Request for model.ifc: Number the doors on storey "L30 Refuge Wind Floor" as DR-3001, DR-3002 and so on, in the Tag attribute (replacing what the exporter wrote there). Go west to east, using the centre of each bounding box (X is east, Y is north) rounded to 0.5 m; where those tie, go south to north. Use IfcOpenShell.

First a look at what the model holds.

```python
import ifcopenshell
import ifcopenshell.util.element
import ifcopenshell.util.placement

model = ifcopenshell.open("model.ifc")
print(model.schema)
storey = next(s for s in model.by_type("IfcBuildingStorey") if s.Name == "L30 Refuge Wind Floor")
doors = [e for e in ifcopenshell.util.element.get_decomposition(storey) if e.is_a("IfcDoor")]
for e in sorted(doors, key=lambda e: e.id()):
    origin = ifcopenshell.util.placement.get_local_placement(e.ObjectPlacement)[:3, 3]
    print(e.id(), e.Tag, e.Name, origin.round(2) + 0.0, sep=" | ")
```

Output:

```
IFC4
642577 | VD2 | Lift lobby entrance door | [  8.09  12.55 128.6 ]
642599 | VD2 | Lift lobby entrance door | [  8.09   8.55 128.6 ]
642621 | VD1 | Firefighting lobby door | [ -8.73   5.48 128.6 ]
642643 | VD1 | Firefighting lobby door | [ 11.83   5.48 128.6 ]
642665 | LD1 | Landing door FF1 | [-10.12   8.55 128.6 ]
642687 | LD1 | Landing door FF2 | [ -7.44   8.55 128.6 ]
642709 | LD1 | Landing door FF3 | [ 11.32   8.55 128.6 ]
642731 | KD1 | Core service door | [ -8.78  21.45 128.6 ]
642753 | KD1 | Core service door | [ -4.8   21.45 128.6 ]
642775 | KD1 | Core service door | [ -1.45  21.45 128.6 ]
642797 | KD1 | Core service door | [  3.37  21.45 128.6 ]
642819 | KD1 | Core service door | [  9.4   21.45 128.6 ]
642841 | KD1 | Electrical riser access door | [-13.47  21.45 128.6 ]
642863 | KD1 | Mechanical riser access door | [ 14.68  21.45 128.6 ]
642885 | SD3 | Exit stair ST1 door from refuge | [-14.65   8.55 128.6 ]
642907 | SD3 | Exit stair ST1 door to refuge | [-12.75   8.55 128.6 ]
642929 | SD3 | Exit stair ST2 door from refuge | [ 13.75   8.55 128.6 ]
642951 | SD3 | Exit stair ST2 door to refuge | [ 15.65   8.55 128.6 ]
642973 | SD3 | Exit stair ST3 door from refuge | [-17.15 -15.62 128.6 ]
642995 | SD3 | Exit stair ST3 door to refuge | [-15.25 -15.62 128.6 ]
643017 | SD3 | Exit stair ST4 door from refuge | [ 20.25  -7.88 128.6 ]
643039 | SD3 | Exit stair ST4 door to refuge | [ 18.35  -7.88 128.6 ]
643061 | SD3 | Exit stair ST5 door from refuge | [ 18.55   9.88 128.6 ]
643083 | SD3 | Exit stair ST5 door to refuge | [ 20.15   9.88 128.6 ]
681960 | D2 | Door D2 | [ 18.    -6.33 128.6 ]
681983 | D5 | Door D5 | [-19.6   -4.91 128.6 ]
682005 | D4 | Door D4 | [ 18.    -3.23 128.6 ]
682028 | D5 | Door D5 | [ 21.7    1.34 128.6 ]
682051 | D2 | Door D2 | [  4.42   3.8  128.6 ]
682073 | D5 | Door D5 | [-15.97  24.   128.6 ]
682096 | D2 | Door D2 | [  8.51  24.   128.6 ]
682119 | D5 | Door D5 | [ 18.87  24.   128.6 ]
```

```python
import ifcopenshell
import ifcopenshell.geom
import ifcopenshell.util.element
import ifcopenshell.util.shape

model = ifcopenshell.open("model.ifc")
settings = ifcopenshell.geom.settings()
settings.set("use-world-coords", True)


def centre(element):
    shape = ifcopenshell.geom.create_shape(settings, element)
    return ifcopenshell.util.shape.get_bbox_centroid(shape.geometry)


storey = next(s for s in model.by_type("IfcBuildingStorey") if s.Name == "L30 Refuge Wind Floor")
doors = [e for e in ifcopenshell.util.element.get_decomposition(storey) if e.is_a("IfcDoor")]

# Insertion points can sit at a corner or the storey origin, so sort by the geometry (in metres).
centres = {e: centre(e) for e in doors}
doors.sort(key=lambda e: (round(centres[e][0] / 0.5), centres[e][1]))

for i, e in enumerate(doors, start=1):
    number = f"DR-30{i:02d}"
    e.Tag = number
    print(e.id(), number)

model.write("model_edited.ifc")
```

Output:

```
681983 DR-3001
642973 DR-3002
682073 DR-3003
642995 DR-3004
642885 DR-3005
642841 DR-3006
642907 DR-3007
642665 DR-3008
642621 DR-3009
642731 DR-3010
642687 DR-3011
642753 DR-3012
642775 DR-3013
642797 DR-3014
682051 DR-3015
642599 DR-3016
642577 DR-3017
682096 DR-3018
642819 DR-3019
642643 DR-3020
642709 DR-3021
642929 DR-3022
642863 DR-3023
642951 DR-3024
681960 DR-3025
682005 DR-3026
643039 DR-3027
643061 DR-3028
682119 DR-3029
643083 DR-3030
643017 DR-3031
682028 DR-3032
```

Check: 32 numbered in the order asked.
